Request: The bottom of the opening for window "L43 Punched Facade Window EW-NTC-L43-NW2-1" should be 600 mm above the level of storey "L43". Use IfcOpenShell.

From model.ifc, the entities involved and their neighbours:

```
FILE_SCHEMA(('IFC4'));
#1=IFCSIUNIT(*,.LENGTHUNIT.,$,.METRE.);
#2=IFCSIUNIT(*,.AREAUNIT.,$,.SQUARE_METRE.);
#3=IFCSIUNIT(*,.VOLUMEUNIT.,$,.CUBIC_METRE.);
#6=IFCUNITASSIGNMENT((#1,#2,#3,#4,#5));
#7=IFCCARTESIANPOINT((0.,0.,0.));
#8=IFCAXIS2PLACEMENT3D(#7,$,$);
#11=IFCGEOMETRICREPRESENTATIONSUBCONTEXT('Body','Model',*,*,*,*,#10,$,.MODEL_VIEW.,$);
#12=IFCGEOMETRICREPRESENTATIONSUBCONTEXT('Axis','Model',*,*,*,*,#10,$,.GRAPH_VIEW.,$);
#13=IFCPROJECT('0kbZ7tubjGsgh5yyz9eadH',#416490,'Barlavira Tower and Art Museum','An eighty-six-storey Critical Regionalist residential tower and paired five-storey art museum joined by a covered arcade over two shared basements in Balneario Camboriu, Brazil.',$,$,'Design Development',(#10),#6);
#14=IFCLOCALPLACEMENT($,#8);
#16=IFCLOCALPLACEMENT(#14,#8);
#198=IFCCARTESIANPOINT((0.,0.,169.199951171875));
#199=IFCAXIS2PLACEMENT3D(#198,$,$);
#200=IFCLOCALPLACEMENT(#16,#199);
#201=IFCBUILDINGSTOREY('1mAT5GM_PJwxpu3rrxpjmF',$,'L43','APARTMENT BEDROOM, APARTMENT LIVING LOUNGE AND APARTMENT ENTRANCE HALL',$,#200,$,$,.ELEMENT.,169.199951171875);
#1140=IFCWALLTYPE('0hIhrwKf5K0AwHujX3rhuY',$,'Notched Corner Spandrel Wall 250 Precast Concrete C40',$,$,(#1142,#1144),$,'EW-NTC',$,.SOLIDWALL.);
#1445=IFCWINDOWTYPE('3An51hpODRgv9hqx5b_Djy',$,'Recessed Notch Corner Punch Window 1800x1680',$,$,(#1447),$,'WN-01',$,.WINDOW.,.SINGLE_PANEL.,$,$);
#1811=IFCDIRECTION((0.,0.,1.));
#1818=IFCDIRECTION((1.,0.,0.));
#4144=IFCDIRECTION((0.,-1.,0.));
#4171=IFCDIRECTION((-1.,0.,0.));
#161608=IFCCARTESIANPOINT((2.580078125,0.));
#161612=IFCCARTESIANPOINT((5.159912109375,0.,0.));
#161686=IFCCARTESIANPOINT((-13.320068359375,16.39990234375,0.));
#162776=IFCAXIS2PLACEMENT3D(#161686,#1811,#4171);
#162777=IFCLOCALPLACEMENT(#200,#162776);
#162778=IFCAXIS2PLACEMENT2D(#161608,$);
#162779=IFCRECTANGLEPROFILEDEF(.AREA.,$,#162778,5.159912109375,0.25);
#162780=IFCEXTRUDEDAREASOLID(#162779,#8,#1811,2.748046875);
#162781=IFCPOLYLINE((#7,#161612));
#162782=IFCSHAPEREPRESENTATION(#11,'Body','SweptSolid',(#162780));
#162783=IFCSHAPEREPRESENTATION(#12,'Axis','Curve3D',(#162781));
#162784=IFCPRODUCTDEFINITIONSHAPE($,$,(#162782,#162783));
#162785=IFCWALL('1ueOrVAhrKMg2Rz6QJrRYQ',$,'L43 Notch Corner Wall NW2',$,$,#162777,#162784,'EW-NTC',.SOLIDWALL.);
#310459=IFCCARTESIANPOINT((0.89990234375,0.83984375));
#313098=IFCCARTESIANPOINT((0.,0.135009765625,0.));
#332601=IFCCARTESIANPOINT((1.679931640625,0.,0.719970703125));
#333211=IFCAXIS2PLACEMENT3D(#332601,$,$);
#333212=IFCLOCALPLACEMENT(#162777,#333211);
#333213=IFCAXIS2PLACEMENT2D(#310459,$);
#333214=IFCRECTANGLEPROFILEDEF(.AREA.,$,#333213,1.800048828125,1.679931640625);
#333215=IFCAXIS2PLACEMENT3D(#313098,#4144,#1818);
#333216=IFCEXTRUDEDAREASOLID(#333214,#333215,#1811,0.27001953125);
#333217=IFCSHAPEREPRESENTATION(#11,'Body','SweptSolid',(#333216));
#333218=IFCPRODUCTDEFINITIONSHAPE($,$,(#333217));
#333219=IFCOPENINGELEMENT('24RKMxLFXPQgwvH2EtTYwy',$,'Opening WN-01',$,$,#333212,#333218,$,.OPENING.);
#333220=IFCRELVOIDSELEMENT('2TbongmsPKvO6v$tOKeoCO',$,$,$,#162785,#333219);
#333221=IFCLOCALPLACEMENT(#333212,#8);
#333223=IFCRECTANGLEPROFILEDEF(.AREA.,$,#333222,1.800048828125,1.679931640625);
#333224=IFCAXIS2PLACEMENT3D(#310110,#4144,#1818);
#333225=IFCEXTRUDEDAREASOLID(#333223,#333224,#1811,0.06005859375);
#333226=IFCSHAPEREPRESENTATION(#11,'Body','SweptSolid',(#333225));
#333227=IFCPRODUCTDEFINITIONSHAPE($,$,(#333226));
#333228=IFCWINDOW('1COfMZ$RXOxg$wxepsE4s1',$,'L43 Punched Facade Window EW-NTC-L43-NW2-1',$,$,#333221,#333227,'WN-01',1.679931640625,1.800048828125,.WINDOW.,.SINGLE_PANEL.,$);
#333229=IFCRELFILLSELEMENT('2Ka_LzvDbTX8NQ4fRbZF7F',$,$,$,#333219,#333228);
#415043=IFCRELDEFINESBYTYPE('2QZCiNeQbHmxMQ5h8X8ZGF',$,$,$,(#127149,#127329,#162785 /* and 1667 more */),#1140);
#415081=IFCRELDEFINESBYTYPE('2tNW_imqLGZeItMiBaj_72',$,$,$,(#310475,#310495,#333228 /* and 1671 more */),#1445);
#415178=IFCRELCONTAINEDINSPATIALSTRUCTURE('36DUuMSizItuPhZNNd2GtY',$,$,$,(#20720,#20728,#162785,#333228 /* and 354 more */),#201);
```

```python
import numpy as np
import ifcopenshell
import ifcopenshell.api.geometry
import ifcopenshell.geom
import ifcopenshell.util.element
import ifcopenshell.util.placement
import ifcopenshell.util.shape
import ifcopenshell.util.unit

model = ifcopenshell.open("model.ifc")
unit_scale = ifcopenshell.util.unit.calculate_unit_scale(model)

window = model.by_guid("1COfMZ$RXOxg$wxepsE4s1")
opening = window.FillsVoids[0].RelatingOpeningElement
storey = ifcopenshell.util.element.get_container(window, ifc_class="IfcBuildingStorey")
level = ifcopenshell.util.placement.get_local_placement(storey.ObjectPlacement)[2, 3]

# The opening's origin need not be at the sill, so measure its lowest point.
shape = ifcopenshell.geom.create_shape(ifcopenshell.geom.settings(), opening)
bottom = ifcopenshell.util.shape.get_shape_bottom_elevation(shape, shape.geometry) / unit_scale
dz = level + 0.6 / unit_scale - bottom

shift = np.array([0.0, 0.0, dz])
# The window is placed relative to its opening, so it follows when the opening moves.
matrix = ifcopenshell.util.placement.get_local_placement(opening.ObjectPlacement)
matrix[:3, 3] += shift
ifcopenshell.api.geometry.edit_object_placement(
    model, product=opening, matrix=matrix, is_si=False, should_transform_children=True
)

print(f"moved by {dz * unit_scale:+.3f} m")

model.write("model_updated.ifc")
```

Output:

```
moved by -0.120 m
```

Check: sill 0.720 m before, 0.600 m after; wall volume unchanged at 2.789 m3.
